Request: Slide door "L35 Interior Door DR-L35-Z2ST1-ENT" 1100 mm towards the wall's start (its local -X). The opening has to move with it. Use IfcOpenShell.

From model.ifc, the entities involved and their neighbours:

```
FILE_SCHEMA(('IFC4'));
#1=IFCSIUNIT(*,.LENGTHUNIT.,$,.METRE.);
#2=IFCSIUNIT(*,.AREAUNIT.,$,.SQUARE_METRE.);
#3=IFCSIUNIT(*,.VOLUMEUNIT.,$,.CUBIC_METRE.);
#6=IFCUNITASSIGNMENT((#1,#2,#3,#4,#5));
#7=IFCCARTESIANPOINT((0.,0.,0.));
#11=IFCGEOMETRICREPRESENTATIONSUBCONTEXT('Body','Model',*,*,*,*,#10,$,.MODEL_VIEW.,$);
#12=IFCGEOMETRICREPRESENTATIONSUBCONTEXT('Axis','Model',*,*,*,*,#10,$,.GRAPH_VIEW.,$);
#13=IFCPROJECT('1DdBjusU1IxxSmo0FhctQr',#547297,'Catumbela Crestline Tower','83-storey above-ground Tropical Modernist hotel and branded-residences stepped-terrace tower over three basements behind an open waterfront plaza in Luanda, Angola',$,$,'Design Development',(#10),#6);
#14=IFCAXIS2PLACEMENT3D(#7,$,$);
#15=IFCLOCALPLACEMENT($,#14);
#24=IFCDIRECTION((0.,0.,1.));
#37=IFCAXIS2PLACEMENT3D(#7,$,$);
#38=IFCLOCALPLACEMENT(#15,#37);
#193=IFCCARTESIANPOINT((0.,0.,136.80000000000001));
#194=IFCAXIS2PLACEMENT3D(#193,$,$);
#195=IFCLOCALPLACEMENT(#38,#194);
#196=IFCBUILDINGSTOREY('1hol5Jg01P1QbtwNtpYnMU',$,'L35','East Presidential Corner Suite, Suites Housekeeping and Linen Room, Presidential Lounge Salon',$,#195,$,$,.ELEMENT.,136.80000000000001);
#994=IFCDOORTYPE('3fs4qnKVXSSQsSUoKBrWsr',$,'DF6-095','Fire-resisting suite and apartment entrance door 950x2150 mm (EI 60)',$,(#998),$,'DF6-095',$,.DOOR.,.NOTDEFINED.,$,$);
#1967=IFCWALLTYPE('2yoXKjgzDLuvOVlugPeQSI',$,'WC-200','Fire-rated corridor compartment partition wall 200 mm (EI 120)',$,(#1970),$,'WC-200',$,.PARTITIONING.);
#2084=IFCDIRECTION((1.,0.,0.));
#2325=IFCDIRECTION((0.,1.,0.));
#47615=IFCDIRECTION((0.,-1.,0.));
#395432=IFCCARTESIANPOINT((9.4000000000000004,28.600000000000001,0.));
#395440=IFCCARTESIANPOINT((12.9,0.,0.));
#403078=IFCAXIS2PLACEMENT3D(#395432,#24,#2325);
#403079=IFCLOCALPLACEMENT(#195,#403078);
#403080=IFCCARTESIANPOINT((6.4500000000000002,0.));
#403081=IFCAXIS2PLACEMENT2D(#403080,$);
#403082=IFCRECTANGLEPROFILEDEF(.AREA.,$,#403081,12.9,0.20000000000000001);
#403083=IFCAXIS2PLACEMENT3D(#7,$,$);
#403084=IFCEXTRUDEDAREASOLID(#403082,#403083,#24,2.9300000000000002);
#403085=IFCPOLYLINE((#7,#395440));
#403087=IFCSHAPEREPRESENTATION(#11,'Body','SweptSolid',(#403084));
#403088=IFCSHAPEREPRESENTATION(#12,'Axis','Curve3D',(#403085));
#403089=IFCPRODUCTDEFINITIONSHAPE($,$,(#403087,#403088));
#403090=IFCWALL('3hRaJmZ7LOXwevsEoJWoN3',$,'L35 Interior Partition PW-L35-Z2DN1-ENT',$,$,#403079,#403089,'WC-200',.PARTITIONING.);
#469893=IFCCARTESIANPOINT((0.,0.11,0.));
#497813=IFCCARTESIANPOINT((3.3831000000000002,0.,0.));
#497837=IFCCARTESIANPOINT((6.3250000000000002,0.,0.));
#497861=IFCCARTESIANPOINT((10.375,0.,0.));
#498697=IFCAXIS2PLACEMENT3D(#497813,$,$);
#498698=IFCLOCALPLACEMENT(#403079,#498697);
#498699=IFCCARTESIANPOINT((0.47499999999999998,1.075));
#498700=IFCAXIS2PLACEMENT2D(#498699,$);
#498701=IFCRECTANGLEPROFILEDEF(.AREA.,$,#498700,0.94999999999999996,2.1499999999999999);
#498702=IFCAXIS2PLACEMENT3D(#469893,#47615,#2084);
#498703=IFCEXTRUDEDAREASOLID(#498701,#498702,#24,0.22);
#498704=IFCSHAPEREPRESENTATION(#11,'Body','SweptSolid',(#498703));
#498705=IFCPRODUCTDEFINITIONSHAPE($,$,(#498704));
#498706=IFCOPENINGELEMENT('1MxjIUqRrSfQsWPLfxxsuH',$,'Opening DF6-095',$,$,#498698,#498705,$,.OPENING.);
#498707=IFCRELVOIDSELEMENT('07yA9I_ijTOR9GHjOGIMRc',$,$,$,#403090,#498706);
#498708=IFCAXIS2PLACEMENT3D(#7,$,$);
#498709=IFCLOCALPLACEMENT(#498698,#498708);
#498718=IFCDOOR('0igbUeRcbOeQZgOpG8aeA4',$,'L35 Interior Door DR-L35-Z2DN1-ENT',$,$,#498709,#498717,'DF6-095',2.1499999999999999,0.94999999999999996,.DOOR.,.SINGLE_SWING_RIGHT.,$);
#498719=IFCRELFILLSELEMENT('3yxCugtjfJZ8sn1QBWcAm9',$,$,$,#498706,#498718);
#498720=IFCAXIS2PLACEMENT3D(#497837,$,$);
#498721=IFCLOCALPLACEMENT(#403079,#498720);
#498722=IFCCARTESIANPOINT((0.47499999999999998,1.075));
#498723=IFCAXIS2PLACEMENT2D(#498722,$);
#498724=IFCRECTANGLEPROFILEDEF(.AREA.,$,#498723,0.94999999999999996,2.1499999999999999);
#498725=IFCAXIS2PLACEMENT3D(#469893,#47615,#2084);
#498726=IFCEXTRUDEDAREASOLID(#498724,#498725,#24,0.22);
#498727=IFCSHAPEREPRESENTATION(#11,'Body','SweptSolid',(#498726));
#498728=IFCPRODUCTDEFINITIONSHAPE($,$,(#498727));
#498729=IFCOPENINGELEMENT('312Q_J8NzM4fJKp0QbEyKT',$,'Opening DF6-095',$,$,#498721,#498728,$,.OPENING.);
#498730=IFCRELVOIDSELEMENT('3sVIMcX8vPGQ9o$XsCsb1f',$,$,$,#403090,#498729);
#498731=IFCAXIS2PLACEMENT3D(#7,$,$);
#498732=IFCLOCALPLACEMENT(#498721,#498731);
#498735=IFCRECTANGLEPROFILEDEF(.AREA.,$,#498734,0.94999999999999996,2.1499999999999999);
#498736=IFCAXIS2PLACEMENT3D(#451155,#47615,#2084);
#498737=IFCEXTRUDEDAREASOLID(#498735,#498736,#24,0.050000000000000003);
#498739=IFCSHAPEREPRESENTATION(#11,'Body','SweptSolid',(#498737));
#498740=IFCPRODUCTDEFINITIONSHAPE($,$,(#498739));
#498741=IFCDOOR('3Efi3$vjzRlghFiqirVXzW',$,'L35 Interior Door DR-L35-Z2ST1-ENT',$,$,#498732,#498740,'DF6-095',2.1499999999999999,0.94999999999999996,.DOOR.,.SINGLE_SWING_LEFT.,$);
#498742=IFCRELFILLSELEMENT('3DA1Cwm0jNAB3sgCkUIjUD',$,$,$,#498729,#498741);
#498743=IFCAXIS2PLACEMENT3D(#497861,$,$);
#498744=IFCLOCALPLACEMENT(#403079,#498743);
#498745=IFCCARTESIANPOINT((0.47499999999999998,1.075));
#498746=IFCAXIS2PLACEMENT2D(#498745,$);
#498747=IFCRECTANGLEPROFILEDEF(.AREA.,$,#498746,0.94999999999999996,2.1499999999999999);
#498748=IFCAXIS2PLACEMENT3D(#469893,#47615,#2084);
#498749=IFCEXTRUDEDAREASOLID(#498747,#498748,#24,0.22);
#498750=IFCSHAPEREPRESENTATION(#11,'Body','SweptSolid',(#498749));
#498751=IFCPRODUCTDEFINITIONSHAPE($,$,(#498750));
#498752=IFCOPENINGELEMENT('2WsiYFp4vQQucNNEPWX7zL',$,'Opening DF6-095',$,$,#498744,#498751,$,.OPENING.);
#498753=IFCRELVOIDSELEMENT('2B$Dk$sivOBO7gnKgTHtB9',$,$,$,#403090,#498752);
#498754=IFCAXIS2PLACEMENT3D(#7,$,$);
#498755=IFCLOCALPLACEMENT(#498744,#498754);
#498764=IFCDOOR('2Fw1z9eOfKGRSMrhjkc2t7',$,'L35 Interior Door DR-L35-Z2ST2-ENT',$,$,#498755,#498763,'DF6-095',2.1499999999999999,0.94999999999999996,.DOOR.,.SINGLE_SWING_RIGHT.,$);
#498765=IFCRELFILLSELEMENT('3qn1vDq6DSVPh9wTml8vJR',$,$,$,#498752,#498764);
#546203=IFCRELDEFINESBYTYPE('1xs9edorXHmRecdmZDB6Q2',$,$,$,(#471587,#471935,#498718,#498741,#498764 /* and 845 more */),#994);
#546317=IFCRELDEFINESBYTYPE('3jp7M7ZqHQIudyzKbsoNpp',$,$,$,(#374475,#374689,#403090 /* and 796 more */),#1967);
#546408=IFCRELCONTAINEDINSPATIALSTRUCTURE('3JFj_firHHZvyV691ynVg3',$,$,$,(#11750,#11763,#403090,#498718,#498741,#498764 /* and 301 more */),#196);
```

```python
import ifcopenshell
import ifcopenshell.api.geometry
import ifcopenshell.util.placement
import ifcopenshell.util.unit

model = ifcopenshell.open("model.ifc")
unit_scale = ifcopenshell.util.unit.calculate_unit_scale(model)

door = model.by_guid("3Efi3$vjzRlghFiqirVXzW")
opening = door.FillsVoids[0].RelatingOpeningElement
wall = opening.VoidsElements[0].RelatingBuildingElement

wall_matrix = ifcopenshell.util.placement.get_local_placement(wall.ObjectPlacement)
shift = wall_matrix[:3, 0] * -1.1 / unit_scale
before = ifcopenshell.util.placement.get_local_placement(door.ObjectPlacement)[:3, 3].copy()

# The door is placed relative to its opening, so it follows when the opening moves.
matrix = ifcopenshell.util.placement.get_local_placement(opening.ObjectPlacement)
matrix[:3, 3] += shift
ifcopenshell.api.geometry.edit_object_placement(
    model, product=opening, matrix=matrix, is_si=False, should_transform_children=True
)

after = ifcopenshell.util.placement.get_local_placement(door.ObjectPlacement)[:3, 3]
print("door moved by", (after - before).round(3) + 0.0)

model.write("model_v2.ifc")
```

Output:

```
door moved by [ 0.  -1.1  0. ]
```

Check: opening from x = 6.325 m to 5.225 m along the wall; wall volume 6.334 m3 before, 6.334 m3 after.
